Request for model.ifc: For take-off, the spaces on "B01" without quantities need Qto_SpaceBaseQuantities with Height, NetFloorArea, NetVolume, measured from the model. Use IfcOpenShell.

First a look at what the model holds.

```python
import ifcopenshell
import ifcopenshell.util.element
import ifcopenshell.util.unit

model = ifcopenshell.open("model.ifc")
print(model.schema)
for unit_type in ("LENGTHUNIT", "AREAUNIT", "VOLUMEUNIT"):
    print(unit_type, ifcopenshell.util.unit.calculate_unit_scale(model, unit_type))
storey = next(s for s in model.by_type("IfcBuildingStorey") if s.Name == "B01")
spaces = [e for e in ifcopenshell.util.element.get_decomposition(storey) if e.is_a("IfcSpace")]
for e in sorted(spaces, key=lambda e: e.id()):
    print(e.id(), e.is_a(), e.Name, list(ifcopenshell.util.element.get_psets(e, qtos_only=True)), sep=" | ")
```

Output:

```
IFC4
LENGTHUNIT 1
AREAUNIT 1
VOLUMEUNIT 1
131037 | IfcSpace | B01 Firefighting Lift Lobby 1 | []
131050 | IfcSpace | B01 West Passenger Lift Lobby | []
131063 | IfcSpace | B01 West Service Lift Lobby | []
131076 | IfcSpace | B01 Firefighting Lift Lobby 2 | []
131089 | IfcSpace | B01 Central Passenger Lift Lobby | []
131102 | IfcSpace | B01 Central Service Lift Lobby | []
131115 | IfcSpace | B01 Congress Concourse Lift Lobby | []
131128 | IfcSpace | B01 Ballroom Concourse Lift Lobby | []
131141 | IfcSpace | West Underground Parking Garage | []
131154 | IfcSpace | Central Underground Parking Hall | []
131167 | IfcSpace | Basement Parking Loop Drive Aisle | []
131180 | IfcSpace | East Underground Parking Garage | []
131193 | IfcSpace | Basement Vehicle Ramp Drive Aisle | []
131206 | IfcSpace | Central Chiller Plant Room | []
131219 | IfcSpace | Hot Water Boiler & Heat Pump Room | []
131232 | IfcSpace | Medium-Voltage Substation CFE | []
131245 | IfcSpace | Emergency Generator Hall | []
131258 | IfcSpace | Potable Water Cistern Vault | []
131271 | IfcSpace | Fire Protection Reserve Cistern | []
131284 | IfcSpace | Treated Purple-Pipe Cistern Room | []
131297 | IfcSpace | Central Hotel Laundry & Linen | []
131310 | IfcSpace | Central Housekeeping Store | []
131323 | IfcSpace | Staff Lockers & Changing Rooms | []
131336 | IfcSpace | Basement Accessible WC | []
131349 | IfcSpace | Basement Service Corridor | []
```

```python
import ifcopenshell
import ifcopenshell.api.pset
import ifcopenshell.geom
import ifcopenshell.util.element
import ifcopenshell.util.shape
import ifcopenshell.util.unit

model = ifcopenshell.open("model.ifc")
unit_scale = ifcopenshell.util.unit.calculate_unit_scale(model)
area_scale = ifcopenshell.util.unit.calculate_unit_scale(model, "AREAUNIT")
volume_scale = ifcopenshell.util.unit.calculate_unit_scale(model, "VOLUMEUNIT")
settings = ifcopenshell.geom.settings()

storey = next(s for s in model.by_type("IfcBuildingStorey") if s.Name == "B01")
spaces = [e for e in ifcopenshell.util.element.get_decomposition(storey) if e.is_a("IfcSpace")]

for e in sorted(spaces, key=lambda e: e.id()):
    if ifcopenshell.util.element.get_psets(e, qtos_only=True, should_inherit=False):
        continue
    # Geometry comes back in metres, in the element's own axes.
    shape = ifcopenshell.geom.create_shape(settings, e)
    values = {
        "Height": ifcopenshell.util.shape.get_z(shape.geometry) / unit_scale,
        "NetFloorArea": ifcopenshell.util.shape.get_footprint_area(shape.geometry) / area_scale,
        "NetVolume": ifcopenshell.util.shape.get_volume(shape.geometry) / volume_scale,
    }
    qto = ifcopenshell.api.pset.add_qto(model, product=e, name="Qto_SpaceBaseQuantities")
    ifcopenshell.api.pset.edit_qto(model, qto=qto, properties=values)
    print(e.id(), {k: round(v, 3) for k, v in values.items()})

model.write("model_updated.ifc")
```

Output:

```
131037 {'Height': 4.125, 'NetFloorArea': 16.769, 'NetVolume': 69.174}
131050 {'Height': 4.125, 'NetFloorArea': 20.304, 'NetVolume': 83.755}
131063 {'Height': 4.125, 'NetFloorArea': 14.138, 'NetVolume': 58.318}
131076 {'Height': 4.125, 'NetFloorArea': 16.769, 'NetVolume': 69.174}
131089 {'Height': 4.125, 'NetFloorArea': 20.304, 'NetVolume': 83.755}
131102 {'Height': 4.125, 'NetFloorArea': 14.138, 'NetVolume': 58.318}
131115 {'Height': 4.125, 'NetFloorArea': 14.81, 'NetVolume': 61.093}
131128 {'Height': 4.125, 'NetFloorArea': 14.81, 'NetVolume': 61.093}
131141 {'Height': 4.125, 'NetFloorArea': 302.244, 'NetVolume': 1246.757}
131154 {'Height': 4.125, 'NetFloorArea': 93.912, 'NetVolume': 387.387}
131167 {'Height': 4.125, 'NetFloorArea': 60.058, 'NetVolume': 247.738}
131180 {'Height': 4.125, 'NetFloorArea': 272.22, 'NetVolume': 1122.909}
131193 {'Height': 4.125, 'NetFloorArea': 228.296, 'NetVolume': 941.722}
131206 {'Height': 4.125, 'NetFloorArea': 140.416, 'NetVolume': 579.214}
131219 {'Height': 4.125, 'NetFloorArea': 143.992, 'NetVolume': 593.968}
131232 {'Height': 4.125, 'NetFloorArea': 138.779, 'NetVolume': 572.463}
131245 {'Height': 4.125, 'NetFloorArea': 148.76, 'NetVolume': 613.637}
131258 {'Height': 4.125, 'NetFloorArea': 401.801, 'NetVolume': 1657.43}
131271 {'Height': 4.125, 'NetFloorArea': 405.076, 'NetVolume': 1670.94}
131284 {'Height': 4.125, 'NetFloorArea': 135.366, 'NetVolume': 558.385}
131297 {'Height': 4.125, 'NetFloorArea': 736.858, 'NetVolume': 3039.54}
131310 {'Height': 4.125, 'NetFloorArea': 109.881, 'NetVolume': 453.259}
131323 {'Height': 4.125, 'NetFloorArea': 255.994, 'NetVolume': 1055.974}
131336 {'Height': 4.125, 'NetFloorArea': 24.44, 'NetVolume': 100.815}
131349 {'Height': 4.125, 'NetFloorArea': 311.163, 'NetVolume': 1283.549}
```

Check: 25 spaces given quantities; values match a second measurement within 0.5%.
